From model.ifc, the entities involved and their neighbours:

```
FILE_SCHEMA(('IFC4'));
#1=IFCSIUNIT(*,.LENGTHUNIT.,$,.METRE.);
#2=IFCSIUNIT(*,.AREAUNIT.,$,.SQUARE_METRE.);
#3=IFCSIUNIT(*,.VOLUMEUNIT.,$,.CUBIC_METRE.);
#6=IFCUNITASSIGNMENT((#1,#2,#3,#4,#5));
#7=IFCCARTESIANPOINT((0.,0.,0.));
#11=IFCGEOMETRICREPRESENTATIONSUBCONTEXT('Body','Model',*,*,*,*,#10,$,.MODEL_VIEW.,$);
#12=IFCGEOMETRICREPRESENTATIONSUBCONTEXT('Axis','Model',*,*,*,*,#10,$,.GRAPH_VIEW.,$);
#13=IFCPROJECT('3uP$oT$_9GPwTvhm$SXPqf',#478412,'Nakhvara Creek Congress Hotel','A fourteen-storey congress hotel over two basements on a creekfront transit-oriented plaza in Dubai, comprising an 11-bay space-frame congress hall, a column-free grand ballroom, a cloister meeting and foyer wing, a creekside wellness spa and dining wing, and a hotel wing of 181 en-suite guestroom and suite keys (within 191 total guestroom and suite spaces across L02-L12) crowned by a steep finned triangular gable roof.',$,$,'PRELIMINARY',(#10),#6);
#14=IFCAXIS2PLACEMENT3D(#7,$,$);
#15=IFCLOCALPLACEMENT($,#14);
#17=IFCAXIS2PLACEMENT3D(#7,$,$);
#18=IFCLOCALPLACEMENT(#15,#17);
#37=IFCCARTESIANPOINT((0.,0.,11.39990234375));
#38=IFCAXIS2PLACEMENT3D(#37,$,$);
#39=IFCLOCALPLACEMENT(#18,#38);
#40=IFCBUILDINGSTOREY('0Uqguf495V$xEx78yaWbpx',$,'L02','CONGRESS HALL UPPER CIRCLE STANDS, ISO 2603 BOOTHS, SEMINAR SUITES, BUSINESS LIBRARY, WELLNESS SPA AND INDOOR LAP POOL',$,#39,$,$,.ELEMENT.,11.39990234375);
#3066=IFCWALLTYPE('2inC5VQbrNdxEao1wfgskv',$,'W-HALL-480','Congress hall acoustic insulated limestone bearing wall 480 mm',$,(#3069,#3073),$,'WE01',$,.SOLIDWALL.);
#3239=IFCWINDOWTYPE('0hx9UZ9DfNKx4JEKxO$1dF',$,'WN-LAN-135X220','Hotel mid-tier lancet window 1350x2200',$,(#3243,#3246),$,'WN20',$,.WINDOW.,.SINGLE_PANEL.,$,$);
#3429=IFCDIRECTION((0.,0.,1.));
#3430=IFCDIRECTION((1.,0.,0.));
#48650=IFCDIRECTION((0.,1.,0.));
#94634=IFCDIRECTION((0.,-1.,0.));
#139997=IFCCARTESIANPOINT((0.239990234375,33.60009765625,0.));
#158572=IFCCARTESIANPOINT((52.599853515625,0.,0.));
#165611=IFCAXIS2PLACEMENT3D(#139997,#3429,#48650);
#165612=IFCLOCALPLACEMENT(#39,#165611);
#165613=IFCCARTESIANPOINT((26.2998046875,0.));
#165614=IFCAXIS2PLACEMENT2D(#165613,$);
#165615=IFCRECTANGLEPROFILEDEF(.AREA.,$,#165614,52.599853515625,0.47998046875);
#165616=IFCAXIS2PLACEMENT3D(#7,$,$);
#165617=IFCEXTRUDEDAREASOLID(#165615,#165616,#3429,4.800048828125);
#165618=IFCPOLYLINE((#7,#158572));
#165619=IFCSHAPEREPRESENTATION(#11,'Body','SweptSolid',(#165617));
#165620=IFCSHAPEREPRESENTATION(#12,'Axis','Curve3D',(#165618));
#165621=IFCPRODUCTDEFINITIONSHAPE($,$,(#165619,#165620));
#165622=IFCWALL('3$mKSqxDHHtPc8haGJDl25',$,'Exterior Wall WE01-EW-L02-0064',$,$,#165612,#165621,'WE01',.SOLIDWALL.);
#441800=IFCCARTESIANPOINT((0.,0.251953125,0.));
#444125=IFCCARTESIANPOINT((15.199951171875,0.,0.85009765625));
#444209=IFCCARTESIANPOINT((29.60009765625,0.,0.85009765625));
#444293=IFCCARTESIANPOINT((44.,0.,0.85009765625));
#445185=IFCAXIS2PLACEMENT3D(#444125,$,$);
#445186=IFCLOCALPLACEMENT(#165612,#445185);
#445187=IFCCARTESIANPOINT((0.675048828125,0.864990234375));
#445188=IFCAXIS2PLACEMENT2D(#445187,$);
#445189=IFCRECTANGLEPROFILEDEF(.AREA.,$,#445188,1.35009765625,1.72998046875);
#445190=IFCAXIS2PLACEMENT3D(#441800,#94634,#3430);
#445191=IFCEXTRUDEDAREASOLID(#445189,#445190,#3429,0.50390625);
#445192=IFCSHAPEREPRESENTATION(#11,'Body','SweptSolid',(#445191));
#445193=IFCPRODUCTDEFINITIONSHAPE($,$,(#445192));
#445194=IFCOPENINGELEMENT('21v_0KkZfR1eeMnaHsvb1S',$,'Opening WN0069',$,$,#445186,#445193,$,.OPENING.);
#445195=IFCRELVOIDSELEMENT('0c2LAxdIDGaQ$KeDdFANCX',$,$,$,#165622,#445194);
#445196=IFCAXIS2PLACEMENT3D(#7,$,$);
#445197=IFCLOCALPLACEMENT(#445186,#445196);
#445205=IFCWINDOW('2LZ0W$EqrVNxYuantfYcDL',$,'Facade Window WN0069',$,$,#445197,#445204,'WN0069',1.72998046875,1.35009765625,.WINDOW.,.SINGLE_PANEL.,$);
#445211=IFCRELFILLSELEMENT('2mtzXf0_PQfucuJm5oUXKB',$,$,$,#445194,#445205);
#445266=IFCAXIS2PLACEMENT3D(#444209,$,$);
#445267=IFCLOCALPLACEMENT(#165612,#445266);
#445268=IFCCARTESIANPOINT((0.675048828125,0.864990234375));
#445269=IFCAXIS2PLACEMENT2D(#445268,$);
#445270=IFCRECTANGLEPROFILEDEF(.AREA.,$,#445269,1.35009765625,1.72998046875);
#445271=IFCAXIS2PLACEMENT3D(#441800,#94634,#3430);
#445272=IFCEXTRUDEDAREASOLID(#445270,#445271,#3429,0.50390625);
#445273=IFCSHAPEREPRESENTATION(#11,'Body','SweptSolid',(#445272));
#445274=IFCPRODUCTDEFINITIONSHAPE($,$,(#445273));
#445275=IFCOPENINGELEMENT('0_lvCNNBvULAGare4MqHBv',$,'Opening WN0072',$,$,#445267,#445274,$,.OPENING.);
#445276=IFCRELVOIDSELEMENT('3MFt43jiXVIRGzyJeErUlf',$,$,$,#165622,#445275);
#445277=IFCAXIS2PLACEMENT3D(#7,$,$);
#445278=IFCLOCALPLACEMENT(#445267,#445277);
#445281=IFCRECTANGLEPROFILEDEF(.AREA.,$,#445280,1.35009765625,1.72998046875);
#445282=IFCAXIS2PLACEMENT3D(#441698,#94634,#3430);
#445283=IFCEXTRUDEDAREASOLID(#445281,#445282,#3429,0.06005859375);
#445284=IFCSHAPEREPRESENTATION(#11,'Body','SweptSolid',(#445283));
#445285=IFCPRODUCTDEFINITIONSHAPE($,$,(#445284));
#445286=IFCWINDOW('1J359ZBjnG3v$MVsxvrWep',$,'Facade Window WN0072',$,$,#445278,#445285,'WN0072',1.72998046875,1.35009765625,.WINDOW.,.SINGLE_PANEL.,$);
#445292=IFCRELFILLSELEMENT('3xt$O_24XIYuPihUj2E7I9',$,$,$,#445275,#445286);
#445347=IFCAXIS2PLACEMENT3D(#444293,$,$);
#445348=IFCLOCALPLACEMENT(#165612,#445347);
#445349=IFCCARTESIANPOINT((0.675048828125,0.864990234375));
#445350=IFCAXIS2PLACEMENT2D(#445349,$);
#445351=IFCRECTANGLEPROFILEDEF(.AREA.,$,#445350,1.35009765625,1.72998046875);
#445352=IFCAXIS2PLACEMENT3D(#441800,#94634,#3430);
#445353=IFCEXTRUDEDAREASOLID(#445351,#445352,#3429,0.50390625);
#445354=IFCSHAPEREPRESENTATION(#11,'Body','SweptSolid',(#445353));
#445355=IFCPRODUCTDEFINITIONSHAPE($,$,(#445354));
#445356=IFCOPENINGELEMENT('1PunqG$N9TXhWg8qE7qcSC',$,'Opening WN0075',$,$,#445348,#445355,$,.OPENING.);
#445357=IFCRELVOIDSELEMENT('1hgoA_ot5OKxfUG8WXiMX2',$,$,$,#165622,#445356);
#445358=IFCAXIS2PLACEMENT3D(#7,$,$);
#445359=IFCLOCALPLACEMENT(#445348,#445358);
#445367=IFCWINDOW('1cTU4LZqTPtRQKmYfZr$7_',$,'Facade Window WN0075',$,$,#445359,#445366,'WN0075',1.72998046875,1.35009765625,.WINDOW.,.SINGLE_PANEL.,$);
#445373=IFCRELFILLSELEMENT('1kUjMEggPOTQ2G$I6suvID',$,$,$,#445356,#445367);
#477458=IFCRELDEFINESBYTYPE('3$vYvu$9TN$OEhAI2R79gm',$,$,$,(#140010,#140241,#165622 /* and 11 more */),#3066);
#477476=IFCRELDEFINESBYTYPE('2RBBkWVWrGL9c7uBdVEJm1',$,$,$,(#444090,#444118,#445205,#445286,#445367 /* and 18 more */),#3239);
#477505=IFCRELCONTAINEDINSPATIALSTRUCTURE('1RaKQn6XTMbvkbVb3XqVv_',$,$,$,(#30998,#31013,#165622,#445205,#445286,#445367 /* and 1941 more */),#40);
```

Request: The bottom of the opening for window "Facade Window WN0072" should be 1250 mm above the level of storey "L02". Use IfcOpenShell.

```python
import numpy as np
import ifcopenshell
import ifcopenshell.api.geometry
import ifcopenshell.geom
import ifcopenshell.util.element
import ifcopenshell.util.placement
import ifcopenshell.util.shape
import ifcopenshell.util.unit

model = ifcopenshell.open("model.ifc")
unit_scale = ifcopenshell.util.unit.calculate_unit_scale(model)

window = model.by_id(445286)
opening = window.FillsVoids[0].RelatingOpeningElement
storey = ifcopenshell.util.element.get_container(window, ifc_class="IfcBuildingStorey")
level = ifcopenshell.util.placement.get_local_placement(storey.ObjectPlacement)[2, 3]

# The opening's origin need not be at the sill, so measure its lowest point.
shape = ifcopenshell.geom.create_shape(ifcopenshell.geom.settings(), opening)
bottom = ifcopenshell.util.shape.get_shape_bottom_elevation(shape, shape.geometry) / unit_scale
dz = level + 1.25 - bottom

shift = np.array([0.0, 0.0, dz])
# The window is placed relative to its opening, so it follows when the opening moves.
matrix = ifcopenshell.util.placement.get_local_placement(opening.ObjectPlacement)
matrix[:3, 3] += shift
ifcopenshell.api.geometry.edit_object_placement(
    model, product=opening, matrix=matrix, is_si=False, should_transform_children=True
)

print(f"moved by {dz * unit_scale:+.3f} m")

model.write("model_v2.ifc")
```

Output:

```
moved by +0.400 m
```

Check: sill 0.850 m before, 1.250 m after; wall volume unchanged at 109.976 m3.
